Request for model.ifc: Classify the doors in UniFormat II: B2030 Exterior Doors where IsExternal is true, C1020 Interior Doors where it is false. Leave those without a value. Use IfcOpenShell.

First a look at what the model holds.

```python
import ifcopenshell
import ifcopenshell.util.element

model = ifcopenshell.open("model.ifc")
print(model.schema)
print("classifications:", [c.Name for c in model.by_type("IfcClassification")])
values = [ifcopenshell.util.element.get_pset(e, "Pset_DoorCommon", "IsExternal") for e in model.by_type("IfcDoor")]
for value in (True, False, None):
    print("IsExternal", value, values.count(value))
```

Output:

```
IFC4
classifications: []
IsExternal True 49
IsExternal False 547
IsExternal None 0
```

```python
import ifcopenshell
import ifcopenshell.api.classification
import ifcopenshell.util.element

model = ifcopenshell.open("model.ifc")

system = ifcopenshell.api.classification.add_classification(model, classification="UniFormat II")

doors = model.by_type("IfcDoor")
external = {e: ifcopenshell.util.element.get_pset(e, "Pset_DoorCommon", "IsExternal") for e in doors}
for flag, code, name in ((True, "B2030", "Exterior Doors"), (False, "C1020", "Interior Doors")):
    products = [e for e in doors if external[e] is flag]
    ifcopenshell.api.classification.add_reference(
        model, products=products, classification=system, identification=code, name=name
    )
    print(code, len(products))

model.write("model-out.ifc")
```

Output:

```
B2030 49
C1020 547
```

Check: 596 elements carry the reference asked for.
